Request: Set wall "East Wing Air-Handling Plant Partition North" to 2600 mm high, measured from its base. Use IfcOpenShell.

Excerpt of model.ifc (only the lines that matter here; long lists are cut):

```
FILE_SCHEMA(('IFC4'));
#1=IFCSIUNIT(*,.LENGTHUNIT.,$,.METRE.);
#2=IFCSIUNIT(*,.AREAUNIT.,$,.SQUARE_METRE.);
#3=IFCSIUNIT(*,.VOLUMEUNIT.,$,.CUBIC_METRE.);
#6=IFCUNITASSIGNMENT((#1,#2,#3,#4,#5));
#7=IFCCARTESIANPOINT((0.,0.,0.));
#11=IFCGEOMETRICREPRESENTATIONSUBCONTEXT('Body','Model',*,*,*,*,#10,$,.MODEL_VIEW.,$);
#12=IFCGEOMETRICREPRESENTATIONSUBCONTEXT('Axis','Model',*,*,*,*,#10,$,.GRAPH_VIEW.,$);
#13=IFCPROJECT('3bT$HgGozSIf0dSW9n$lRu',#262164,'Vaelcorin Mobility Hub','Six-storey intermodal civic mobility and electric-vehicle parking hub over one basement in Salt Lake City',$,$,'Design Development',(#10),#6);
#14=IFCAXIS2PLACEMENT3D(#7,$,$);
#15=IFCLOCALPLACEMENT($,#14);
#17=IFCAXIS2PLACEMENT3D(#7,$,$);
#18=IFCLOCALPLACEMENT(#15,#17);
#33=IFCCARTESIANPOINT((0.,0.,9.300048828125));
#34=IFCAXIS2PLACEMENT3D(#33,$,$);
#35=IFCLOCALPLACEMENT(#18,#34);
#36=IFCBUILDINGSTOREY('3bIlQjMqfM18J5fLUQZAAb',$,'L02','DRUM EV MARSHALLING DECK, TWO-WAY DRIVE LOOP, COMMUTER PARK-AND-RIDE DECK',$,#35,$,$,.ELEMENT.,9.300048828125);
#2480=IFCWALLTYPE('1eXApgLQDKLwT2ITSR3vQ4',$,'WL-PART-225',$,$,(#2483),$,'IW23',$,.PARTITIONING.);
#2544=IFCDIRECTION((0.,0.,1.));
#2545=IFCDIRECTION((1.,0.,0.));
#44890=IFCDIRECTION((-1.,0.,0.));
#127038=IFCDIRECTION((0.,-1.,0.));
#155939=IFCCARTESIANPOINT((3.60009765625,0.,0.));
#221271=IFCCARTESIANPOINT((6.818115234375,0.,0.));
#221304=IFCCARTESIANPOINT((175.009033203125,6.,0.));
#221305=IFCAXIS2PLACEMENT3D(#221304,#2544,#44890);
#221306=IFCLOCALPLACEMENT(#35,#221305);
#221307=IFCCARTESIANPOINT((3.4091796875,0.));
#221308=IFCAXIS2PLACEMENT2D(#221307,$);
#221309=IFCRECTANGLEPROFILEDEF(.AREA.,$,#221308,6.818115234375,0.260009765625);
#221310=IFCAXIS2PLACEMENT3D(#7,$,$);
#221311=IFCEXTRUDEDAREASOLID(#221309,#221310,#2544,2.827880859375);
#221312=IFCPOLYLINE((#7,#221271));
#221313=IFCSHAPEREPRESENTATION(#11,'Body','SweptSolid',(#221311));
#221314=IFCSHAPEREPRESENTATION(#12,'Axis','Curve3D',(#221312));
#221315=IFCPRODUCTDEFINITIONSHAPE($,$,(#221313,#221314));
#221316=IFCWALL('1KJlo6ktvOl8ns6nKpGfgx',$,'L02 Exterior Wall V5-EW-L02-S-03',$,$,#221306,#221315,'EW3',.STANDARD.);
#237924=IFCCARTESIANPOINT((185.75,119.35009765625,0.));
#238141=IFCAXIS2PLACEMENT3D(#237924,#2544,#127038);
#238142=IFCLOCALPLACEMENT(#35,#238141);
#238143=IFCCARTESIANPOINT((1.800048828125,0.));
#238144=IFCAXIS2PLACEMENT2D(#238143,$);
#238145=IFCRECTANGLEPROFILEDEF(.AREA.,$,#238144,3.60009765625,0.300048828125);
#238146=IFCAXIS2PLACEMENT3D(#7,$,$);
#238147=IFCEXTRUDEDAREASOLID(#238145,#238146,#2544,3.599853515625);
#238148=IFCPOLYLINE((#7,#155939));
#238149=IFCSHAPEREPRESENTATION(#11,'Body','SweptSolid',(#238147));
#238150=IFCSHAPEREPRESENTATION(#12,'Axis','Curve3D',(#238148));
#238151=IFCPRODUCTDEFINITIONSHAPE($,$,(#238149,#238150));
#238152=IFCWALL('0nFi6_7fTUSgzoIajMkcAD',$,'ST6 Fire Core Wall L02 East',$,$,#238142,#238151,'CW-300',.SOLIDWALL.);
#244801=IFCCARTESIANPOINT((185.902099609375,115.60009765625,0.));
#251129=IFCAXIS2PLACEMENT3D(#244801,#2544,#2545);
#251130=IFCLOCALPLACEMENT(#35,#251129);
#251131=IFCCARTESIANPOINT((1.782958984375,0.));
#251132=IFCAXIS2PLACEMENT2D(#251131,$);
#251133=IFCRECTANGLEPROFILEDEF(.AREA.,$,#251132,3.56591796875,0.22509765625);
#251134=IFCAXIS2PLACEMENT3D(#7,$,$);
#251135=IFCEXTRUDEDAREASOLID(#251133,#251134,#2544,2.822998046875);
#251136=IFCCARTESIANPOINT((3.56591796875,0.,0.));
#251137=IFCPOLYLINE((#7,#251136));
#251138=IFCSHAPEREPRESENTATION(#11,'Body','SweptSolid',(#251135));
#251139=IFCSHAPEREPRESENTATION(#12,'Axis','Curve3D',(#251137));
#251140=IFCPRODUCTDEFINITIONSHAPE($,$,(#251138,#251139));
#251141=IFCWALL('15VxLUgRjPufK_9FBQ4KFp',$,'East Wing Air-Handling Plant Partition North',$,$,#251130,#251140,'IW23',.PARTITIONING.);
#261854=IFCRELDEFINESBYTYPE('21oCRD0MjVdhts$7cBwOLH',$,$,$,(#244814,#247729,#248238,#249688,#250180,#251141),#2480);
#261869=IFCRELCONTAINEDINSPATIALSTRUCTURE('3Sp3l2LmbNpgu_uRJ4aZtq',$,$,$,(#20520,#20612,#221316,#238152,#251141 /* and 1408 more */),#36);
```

```python
import ifcopenshell
import ifcopenshell.geom
import ifcopenshell.util.representation
import ifcopenshell.util.shape

model = ifcopenshell.open("model.ifc")
settings = ifcopenshell.geom.settings()


def volume(element):
    """Net volume in cubic metres, openings subtracted."""
    shape = ifcopenshell.geom.create_shape(settings, element)
    return ifcopenshell.util.shape.get_volume(shape.geometry)


wall = model.by_guid("15VxLUgRjPufK_9FBQ4KFp")
before = volume(wall)

body = ifcopenshell.util.representation.get_representation(wall, "Model", "Body")
solid = body.Items[0]
old_height = solid.Depth
solid.Depth = 2.6
after = volume(wall)

print(f"height {old_height:g} -> {solid.Depth:g}, volume {before:.3f} -> {after:.3f} m3")

model.write("model_v2.ifc")
```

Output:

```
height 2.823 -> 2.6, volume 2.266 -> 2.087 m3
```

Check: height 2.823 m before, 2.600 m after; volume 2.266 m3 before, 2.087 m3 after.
